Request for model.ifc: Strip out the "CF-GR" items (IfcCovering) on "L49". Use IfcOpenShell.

First a look at what the model holds.

```python
import ifcopenshell
import ifcopenshell.util.element

model = ifcopenshell.open("model.ifc")
print(model.schema)
storey = next(s for s in model.by_type("IfcBuildingStorey") if s.Name == "L49")
coverings = [e for e in ifcopenshell.util.element.get_decomposition(storey) if e.is_a("IfcCovering")]
seen = {}
for e in coverings:
    element_type = ifcopenshell.util.element.get_type(e)
    name = element_type.Name if element_type not in (None, e) else None
    seen[name] = seen.get(name, 0) + 1
for name, count in sorted(seen.items(), key=str):
    print(count, "x", name)
```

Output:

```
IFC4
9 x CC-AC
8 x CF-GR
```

```python
import ifcopenshell
import ifcopenshell.api.root
import ifcopenshell.util.element

model = ifcopenshell.open("model.ifc")

storey = next(s for s in model.by_type("IfcBuildingStorey") if s.Name == "L49")
coverings = [e for e in ifcopenshell.util.element.get_decomposition(storey) if e.is_a("IfcCovering")]
targets = [e for e in coverings if (t := ifcopenshell.util.element.get_type(e)) not in (None, e) and t.Name == "CF-GR"]

for e in targets:
    ifcopenshell.api.root.remove_product(model, product=e)
print(len(targets), "removed")

model.write("model_updated.ifc")
```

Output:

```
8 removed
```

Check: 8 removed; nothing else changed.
